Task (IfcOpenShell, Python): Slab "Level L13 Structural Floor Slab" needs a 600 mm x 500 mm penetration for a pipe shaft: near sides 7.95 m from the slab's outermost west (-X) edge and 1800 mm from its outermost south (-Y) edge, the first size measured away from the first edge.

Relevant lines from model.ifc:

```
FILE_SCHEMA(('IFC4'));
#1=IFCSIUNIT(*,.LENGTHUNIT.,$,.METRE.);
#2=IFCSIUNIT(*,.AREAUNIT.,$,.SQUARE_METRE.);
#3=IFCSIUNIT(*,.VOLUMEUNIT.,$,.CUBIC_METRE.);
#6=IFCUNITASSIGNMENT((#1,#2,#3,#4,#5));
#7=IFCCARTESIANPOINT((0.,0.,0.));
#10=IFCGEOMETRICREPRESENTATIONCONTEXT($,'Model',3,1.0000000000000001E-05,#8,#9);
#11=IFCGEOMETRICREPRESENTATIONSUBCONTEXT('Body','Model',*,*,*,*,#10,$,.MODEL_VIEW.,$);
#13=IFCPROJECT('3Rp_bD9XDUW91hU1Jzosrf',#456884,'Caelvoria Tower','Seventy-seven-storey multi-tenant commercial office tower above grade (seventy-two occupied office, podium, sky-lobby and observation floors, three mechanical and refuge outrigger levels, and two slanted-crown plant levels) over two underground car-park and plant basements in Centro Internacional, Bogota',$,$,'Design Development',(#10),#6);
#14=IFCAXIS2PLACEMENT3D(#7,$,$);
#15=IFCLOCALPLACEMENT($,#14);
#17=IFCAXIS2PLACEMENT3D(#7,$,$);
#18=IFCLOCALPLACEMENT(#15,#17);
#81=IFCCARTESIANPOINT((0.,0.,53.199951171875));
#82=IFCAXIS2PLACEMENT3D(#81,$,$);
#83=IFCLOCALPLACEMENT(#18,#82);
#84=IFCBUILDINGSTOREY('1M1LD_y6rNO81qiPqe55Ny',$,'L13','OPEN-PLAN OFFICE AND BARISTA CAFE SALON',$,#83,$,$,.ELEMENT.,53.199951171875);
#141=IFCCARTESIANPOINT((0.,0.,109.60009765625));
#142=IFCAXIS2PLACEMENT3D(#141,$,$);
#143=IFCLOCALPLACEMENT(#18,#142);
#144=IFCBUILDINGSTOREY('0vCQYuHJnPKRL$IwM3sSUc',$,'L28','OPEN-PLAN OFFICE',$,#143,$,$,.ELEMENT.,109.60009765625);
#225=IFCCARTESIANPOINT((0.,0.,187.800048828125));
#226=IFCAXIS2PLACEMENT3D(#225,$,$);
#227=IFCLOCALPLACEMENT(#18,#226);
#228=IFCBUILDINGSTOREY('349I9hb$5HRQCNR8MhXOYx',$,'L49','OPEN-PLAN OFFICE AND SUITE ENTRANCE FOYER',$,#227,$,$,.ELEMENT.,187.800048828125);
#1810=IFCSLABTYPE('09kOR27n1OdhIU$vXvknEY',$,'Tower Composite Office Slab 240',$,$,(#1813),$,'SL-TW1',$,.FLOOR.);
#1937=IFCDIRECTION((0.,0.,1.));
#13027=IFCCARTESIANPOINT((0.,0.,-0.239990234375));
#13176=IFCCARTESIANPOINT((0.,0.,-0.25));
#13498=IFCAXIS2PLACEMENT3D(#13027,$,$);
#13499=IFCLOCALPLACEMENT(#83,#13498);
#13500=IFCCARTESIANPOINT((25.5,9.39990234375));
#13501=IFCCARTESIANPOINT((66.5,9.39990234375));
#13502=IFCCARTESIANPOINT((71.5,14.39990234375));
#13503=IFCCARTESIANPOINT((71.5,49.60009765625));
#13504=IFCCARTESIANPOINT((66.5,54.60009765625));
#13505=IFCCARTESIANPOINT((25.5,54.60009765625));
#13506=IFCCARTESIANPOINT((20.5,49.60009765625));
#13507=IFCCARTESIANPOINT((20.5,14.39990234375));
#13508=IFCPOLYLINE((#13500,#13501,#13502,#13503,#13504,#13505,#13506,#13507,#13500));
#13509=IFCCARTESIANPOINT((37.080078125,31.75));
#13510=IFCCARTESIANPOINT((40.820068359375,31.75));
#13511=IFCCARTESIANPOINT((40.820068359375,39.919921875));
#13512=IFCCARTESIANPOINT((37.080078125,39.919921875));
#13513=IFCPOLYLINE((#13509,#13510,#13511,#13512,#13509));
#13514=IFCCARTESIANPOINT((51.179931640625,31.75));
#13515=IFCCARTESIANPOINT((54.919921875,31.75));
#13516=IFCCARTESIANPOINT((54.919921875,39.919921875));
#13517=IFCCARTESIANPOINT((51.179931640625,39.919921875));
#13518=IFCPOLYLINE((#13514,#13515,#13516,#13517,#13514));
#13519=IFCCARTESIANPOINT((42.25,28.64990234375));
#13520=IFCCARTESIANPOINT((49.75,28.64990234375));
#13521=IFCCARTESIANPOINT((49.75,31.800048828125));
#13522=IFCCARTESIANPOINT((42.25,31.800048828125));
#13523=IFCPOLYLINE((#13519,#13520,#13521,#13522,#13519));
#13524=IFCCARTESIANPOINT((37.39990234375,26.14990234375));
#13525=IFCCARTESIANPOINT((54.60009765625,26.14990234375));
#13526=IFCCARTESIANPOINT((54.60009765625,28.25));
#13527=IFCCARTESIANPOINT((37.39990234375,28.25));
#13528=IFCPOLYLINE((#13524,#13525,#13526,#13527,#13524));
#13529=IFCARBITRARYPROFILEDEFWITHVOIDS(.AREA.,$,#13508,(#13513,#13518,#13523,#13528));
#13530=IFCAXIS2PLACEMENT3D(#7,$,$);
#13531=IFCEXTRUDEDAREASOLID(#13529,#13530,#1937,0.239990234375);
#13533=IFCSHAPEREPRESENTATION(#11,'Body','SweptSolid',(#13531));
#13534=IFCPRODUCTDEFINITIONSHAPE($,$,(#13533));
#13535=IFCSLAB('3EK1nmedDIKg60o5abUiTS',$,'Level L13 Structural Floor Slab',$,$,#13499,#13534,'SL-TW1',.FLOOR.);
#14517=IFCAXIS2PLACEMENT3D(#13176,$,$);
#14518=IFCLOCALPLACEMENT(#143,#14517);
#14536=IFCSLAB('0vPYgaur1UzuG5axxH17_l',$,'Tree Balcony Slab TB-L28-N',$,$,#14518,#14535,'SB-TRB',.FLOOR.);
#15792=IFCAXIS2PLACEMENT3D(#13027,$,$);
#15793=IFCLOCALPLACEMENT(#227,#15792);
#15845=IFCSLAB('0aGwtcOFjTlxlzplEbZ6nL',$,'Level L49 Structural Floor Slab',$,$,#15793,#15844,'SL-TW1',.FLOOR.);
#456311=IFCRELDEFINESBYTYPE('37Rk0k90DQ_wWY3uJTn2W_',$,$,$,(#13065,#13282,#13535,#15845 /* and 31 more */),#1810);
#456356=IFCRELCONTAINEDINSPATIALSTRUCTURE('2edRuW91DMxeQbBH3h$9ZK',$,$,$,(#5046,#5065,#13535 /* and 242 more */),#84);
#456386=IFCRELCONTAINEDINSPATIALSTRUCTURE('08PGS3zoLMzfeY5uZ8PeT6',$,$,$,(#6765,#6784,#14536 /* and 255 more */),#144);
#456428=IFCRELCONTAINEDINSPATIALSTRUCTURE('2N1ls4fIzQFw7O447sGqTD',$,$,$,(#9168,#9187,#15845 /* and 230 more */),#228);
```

```python
import numpy as np
import ifcopenshell
import ifcopenshell.api.feature
import ifcopenshell.api.geometry
import ifcopenshell.api.root
import ifcopenshell.geom
import ifcopenshell.util.placement
import ifcopenshell.util.representation
import ifcopenshell.util.shape
import ifcopenshell.util.unit

model = ifcopenshell.open("model.ifc")
unit_scale = ifcopenshell.util.unit.calculate_unit_scale(model)
settings = ifcopenshell.geom.settings()


def volume(element):
    """Net volume in cubic metres, openings subtracted."""
    shape = ifcopenshell.geom.create_shape(settings, element)
    return ifcopenshell.util.shape.get_volume(shape.geometry)


slab = model.by_guid("3EK1nmedDIKg60o5abUiTS")
before = volume(slab)

# Extent in the slab's own axes, in metres. The edges named are its -X and -Y sides.
slab_shape = ifcopenshell.geom.create_shape(settings, slab)
vertices = ifcopenshell.util.shape.get_vertices(slab_shape.geometry)
x_min, y_min, bottom = vertices.min(axis=0)
top = vertices[:, 2].max()

opening = ifcopenshell.api.root.create_entity(model, ifc_class="IfcOpeningElement", name="Pipe shaft opening", predefined_type="OPENING")
context = ifcopenshell.util.representation.get_context(model, "Model", "Body", "MODEL_VIEW")
width, depth = 0.6, 0.5
outline = [(0.0, 0.0), (width, 0.0), (width, depth), (0.0, depth), (0.0, 0.0)]
# Overshoot both faces by 50 mm so the cut is clean.
shape = ifcopenshell.api.geometry.add_slab_representation(
    model, context=context, depth=top - bottom + 0.1, polyline=outline
)
ifcopenshell.api.geometry.assign_representation(model, product=opening, representation=shape)

matrix = ifcopenshell.util.placement.get_local_placement(slab.ObjectPlacement)
matrix[:, 3] = matrix @ np.append(np.array([x_min + 7.95, y_min + 1.8, bottom - 0.05]) / unit_scale, 1.0)
ifcopenshell.api.geometry.edit_object_placement(model, product=opening, matrix=matrix, is_si=False)
ifcopenshell.api.feature.add_feature(model, feature=opening, element=slab)

after = volume(slab)

print(f"slab volume {before:.3f} -> {after:.3f} m3")

model.write("model_updated.ifc")
```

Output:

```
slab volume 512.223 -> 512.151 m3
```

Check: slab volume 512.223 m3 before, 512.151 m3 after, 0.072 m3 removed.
